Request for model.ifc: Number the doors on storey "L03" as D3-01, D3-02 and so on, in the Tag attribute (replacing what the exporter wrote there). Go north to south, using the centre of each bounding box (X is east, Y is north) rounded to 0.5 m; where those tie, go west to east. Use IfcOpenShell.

First a look at what the model holds.

```python
import ifcopenshell
import ifcopenshell.util.element
import ifcopenshell.util.placement

model = ifcopenshell.open("model.ifc")
print(model.schema)
storey = next(s for s in model.by_type("IfcBuildingStorey") if s.Name == "L03")
doors = [e for e in ifcopenshell.util.element.get_decomposition(storey) if e.is_a("IfcDoor")]
for e in sorted(doors, key=lambda e: e.id()):
    origin = ifcopenshell.util.placement.get_local_placement(e.ObjectPlacement)[:3, 3]
    print(e.id(), e.Tag, e.Name, origin.round(2) + 0.0, sep=" | ")
```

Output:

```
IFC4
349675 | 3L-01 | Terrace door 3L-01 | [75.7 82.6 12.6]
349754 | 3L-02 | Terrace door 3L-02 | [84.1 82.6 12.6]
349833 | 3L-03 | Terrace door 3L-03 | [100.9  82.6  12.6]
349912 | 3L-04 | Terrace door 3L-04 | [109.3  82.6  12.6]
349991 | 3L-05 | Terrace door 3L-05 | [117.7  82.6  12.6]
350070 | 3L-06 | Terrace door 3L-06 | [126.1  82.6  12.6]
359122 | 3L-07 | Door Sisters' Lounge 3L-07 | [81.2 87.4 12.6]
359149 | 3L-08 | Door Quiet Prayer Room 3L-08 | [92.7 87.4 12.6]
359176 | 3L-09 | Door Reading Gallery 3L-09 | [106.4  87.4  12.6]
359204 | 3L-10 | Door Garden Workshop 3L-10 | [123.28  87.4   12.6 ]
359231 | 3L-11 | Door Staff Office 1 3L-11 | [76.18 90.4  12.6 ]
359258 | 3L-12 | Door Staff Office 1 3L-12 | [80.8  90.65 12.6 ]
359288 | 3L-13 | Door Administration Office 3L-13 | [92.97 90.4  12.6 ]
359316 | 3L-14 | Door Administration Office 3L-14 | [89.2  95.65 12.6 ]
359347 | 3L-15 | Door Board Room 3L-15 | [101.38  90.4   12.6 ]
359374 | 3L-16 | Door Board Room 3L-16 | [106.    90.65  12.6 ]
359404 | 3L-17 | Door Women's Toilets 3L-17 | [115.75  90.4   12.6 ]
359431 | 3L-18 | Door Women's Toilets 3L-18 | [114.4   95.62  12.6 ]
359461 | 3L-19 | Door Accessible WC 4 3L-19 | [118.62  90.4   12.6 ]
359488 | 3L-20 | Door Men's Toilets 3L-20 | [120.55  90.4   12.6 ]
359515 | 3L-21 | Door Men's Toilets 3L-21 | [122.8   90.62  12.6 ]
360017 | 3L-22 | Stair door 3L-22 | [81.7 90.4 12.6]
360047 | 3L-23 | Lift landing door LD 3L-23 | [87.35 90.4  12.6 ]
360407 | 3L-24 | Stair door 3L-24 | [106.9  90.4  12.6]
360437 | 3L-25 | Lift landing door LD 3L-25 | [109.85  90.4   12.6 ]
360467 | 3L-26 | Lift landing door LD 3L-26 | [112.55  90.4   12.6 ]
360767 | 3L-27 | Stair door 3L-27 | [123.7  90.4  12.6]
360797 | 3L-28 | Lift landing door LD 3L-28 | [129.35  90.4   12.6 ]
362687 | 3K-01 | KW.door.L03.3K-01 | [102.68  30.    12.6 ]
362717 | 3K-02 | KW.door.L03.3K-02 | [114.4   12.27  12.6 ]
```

```python
import ifcopenshell
import ifcopenshell.geom
import ifcopenshell.util.element
import ifcopenshell.util.shape

model = ifcopenshell.open("model.ifc")
settings = ifcopenshell.geom.settings()
settings.set("use-world-coords", True)


def centre(element):
    shape = ifcopenshell.geom.create_shape(settings, element)
    return ifcopenshell.util.shape.get_bbox_centroid(shape.geometry)


storey = next(s for s in model.by_type("IfcBuildingStorey") if s.Name == "L03")
doors = [e for e in ifcopenshell.util.element.get_decomposition(storey) if e.is_a("IfcDoor")]

# Insertion points can sit at a corner or the storey origin, so sort by the geometry (in metres).
centres = {e: centre(e) for e in doors}
doors.sort(key=lambda e: (-round(centres[e][1] / 0.5), centres[e][0]))

for i, e in enumerate(doors, start=1):
    number = f"D3-{i:02d}"
    e.Tag = number
    print(e.id(), number)

model.write("model_rev.ifc")
```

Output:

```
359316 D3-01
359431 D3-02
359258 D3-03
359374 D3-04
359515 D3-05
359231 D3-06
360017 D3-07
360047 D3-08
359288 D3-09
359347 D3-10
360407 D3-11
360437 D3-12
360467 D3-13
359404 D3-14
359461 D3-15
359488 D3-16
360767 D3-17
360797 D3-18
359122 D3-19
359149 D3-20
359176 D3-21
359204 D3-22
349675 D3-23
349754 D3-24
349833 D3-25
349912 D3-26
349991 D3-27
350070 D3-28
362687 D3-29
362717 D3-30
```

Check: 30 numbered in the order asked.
